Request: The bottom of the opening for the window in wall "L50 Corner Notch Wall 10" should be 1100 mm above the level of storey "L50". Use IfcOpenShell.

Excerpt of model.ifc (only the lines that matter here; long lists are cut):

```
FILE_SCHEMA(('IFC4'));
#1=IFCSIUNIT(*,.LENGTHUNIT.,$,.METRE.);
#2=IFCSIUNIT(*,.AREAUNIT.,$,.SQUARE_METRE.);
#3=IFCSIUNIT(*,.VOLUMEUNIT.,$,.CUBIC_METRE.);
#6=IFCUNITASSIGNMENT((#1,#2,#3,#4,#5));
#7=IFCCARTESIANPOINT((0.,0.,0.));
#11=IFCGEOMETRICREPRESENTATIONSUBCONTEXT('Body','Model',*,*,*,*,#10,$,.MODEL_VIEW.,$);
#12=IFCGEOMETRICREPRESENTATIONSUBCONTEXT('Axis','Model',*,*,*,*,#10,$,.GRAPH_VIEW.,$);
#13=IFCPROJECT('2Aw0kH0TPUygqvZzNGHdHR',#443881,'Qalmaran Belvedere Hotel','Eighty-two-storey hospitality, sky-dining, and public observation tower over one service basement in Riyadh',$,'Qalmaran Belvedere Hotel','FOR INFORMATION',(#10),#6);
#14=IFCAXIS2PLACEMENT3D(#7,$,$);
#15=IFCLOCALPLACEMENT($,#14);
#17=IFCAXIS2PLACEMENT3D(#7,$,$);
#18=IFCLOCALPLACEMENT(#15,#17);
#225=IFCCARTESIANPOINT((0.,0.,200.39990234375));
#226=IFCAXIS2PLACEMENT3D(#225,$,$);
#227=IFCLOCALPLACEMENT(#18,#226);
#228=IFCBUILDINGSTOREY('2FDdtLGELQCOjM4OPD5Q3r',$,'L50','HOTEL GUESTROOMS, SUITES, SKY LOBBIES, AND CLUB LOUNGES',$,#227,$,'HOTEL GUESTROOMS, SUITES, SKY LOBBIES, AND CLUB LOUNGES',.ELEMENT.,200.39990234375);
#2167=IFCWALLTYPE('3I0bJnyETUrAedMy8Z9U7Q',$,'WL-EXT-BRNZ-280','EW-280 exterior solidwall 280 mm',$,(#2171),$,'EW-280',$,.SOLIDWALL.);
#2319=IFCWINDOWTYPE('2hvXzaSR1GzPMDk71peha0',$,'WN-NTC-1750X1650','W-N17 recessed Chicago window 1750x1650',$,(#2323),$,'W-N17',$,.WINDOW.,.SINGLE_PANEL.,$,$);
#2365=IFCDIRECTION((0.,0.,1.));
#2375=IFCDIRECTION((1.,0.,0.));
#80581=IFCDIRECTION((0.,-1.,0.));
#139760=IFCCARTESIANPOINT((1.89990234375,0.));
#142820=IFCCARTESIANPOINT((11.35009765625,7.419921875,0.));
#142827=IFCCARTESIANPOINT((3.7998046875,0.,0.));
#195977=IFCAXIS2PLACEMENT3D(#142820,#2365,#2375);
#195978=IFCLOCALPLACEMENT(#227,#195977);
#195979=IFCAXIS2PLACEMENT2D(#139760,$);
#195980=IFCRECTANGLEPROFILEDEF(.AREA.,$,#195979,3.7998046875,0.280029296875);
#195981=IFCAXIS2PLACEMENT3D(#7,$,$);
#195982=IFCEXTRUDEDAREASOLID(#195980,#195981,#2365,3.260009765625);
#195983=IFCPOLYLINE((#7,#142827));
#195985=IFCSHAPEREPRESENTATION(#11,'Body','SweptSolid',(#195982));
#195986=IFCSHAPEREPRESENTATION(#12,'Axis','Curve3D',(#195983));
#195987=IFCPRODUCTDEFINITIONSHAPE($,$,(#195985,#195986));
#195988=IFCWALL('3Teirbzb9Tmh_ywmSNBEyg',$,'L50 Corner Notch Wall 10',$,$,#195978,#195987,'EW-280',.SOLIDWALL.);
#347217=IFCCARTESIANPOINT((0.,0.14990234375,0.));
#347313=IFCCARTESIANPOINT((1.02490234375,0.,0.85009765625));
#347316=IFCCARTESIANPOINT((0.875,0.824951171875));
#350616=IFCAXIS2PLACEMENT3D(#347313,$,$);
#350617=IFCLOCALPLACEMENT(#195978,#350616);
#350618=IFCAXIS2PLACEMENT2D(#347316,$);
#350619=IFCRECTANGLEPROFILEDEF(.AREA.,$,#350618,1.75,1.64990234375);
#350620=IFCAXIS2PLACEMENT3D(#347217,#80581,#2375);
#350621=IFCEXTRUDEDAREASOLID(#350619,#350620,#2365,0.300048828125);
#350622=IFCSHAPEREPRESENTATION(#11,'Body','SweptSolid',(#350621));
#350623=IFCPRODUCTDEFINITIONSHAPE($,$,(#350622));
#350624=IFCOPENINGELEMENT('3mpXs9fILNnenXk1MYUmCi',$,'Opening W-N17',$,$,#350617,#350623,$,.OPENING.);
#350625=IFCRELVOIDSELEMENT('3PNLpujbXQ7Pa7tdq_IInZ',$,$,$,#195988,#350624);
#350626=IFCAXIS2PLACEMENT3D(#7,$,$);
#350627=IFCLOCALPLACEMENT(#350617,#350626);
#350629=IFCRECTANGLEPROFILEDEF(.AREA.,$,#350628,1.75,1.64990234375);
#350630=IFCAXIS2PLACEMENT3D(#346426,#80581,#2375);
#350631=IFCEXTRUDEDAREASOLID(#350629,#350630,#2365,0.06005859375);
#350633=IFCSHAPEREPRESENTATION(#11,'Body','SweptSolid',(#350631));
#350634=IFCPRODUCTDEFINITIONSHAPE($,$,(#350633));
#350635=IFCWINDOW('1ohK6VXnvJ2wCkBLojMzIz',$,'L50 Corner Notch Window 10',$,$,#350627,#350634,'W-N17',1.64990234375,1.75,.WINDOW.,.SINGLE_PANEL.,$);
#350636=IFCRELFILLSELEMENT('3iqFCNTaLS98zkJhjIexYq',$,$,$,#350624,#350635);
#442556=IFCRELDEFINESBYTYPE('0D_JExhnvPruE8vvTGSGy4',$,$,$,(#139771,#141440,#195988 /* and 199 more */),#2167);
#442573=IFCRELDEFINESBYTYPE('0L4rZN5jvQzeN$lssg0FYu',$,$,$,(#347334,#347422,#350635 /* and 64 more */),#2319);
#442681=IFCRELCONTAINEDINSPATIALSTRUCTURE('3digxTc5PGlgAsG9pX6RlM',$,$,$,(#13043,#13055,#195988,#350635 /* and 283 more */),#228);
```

```python
import numpy as np
import ifcopenshell
import ifcopenshell.api.geometry
import ifcopenshell.geom
import ifcopenshell.util.element
import ifcopenshell.util.placement
import ifcopenshell.util.shape
import ifcopenshell.util.unit

model = ifcopenshell.open("model.ifc")
unit_scale = ifcopenshell.util.unit.calculate_unit_scale(model)

window = model.by_guid("1ohK6VXnvJ2wCkBLojMzIz")
opening = window.FillsVoids[0].RelatingOpeningElement
storey = ifcopenshell.util.element.get_container(window, ifc_class="IfcBuildingStorey")
level = ifcopenshell.util.placement.get_local_placement(storey.ObjectPlacement)[2, 3]

# The opening's origin need not be at the sill, so measure its lowest point.
shape = ifcopenshell.geom.create_shape(ifcopenshell.geom.settings(), opening)
bottom = ifcopenshell.util.shape.get_shape_bottom_elevation(shape, shape.geometry) / unit_scale
dz = level + 1.1 / unit_scale - bottom

shift = np.array([0.0, 0.0, dz])
# The window is placed relative to its opening, so it follows when the opening moves.
matrix = ifcopenshell.util.placement.get_local_placement(opening.ObjectPlacement)
matrix[:3, 3] += shift
ifcopenshell.api.geometry.edit_object_placement(
    model, product=opening, matrix=matrix, is_si=False, should_transform_children=True
)

print(f"moved by {dz * unit_scale:+.3f} m")

model.write("model_rev.ifc")
```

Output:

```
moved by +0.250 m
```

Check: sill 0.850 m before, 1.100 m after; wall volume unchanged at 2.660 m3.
